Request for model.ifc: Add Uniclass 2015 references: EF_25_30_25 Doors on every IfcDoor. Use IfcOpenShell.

First a look at what the model holds.

```python
import ifcopenshell

model = ifcopenshell.open("model.ifc")
print(model.schema)
print("classifications:", [c.Name for c in model.by_type("IfcClassification")])
for ifc_class in ("IfcDoor", "IfcRoof", "IfcStair", "IfcWall", "IfcWindow"):
    print(ifc_class, len(model.by_type(ifc_class)))
```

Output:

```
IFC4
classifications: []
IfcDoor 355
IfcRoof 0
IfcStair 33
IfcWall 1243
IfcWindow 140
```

```python
import ifcopenshell
import ifcopenshell.api.classification

model = ifcopenshell.open("model.ifc")

system = ifcopenshell.api.classification.add_classification(model, classification="Uniclass 2015")

codes = {
    "IfcDoor": ("EF_25_30_25", "Doors"),
}
for ifc_class, (code, name) in codes.items():
    products = model.by_type(ifc_class)
    ifcopenshell.api.classification.add_reference(
        model, products=products, classification=system, identification=code, name=name
    )
    print(code, len(products))

model.write("model_edited.ifc")
```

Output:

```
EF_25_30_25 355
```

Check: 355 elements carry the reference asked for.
